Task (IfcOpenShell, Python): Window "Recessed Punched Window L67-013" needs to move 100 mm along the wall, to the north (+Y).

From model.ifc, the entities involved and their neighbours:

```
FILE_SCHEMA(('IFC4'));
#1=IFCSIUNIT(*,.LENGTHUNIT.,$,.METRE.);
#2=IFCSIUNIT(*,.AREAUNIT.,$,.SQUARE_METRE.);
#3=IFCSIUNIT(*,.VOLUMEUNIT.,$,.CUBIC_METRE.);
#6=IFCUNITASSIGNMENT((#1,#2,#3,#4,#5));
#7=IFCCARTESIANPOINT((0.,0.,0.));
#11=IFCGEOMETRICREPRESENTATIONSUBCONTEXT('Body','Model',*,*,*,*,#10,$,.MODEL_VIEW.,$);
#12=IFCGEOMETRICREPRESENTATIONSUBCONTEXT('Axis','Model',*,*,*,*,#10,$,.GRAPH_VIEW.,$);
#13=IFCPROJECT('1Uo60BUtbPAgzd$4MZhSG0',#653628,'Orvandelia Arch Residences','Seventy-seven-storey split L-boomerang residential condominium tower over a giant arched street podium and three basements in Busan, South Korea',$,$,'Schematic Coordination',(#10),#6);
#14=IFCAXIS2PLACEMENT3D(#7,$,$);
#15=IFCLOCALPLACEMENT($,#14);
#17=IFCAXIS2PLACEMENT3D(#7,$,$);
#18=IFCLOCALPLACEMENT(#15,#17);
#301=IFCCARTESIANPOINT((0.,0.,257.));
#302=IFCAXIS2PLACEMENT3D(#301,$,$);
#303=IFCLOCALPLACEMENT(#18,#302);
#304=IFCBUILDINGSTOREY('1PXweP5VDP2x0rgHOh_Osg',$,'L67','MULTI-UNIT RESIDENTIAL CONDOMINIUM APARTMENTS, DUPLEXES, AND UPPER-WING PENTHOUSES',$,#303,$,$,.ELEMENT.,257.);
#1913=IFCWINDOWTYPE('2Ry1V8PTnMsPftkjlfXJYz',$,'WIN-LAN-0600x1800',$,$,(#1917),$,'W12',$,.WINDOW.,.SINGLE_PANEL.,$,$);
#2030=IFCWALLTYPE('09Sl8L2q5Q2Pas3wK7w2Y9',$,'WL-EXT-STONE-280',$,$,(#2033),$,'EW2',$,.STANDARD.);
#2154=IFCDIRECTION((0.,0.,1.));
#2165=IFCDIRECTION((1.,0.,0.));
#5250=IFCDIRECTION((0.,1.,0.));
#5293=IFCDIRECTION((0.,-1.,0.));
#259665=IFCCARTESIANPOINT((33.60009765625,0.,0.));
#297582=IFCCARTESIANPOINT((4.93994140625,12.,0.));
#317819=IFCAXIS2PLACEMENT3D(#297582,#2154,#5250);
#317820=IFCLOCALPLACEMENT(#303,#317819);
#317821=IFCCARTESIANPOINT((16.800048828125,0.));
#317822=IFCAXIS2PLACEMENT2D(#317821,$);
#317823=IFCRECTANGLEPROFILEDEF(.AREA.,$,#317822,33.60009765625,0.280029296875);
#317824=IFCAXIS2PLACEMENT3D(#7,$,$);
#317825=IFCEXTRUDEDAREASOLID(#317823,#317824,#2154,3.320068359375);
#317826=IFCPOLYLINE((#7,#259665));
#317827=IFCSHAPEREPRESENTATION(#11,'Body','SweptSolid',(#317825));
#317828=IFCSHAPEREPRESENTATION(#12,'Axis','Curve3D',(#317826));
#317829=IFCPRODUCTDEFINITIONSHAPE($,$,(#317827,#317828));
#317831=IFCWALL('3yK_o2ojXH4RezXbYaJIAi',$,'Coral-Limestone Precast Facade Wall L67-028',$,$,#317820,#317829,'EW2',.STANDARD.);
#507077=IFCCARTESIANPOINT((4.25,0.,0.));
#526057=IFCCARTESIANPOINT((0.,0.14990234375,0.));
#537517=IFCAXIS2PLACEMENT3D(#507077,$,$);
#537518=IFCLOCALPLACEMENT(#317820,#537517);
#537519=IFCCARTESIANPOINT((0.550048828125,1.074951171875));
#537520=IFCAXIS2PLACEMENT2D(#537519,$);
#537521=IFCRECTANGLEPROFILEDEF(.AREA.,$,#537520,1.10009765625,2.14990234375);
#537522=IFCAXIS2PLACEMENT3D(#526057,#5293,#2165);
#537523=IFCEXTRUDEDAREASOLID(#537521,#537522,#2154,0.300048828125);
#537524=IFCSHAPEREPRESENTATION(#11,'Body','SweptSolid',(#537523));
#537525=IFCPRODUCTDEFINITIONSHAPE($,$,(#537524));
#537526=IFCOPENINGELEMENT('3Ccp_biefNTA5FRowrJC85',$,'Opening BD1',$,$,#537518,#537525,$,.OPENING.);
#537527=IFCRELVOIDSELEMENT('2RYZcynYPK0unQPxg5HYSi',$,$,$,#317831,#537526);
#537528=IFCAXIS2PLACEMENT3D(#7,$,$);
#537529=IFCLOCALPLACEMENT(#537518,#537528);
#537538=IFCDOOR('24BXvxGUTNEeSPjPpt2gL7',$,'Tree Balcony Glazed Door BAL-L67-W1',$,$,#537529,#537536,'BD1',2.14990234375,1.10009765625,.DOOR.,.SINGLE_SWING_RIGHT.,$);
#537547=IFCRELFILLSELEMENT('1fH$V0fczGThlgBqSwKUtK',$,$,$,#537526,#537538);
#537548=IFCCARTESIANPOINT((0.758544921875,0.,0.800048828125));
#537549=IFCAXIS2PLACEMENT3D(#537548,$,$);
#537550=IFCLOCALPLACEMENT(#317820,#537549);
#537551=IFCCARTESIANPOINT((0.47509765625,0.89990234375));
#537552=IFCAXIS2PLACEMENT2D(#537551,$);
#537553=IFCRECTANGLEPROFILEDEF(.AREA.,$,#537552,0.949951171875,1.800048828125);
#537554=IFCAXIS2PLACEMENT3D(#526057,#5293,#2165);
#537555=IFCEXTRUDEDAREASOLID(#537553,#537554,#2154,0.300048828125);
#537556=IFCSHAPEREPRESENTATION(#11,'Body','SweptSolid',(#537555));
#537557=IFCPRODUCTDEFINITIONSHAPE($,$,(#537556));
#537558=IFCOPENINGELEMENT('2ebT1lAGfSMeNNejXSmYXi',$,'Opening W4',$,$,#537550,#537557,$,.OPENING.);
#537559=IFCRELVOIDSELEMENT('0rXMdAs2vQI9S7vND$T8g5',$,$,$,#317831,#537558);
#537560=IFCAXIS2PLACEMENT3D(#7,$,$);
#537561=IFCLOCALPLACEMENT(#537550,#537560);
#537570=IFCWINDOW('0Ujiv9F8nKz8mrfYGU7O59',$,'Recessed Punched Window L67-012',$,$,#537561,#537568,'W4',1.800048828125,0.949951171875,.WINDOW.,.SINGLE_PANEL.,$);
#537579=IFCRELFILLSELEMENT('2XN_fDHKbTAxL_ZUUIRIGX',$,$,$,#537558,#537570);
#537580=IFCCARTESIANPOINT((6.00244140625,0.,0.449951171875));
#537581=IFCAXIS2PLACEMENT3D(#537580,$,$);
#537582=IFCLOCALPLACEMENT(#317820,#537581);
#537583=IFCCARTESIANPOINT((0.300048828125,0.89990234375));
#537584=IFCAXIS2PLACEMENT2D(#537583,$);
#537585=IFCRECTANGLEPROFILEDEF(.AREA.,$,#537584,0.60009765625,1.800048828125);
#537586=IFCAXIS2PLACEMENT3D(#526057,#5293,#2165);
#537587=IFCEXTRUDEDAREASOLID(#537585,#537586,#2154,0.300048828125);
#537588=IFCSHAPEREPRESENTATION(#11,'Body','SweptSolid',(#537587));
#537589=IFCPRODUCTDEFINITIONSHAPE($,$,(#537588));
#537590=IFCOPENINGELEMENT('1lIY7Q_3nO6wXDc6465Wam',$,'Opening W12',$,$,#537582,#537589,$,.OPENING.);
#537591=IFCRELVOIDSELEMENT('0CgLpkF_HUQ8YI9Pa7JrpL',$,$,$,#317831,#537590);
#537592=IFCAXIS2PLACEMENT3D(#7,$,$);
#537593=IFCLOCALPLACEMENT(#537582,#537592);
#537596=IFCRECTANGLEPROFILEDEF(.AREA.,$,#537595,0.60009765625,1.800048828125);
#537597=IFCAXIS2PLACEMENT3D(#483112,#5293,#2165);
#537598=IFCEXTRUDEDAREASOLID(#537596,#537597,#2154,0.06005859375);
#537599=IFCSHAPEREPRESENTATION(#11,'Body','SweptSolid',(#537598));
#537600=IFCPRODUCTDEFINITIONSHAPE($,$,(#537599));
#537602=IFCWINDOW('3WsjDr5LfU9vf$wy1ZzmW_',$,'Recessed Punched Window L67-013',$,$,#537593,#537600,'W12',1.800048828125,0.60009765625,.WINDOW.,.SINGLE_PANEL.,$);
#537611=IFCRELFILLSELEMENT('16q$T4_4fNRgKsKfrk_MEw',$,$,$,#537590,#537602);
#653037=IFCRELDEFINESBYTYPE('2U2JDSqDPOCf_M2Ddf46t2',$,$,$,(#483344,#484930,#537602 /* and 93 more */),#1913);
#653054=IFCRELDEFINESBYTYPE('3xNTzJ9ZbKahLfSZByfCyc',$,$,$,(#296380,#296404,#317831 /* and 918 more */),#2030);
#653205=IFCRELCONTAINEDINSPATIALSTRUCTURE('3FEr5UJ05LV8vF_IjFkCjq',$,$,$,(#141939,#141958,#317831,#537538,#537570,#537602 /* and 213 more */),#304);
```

```python
import ifcopenshell
import ifcopenshell.api.geometry
import ifcopenshell.util.placement

model = ifcopenshell.open("model.ifc")

window = model.by_guid("3WsjDr5LfU9vf$wy1ZzmW_")
opening = window.FillsVoids[0].RelatingOpeningElement
wall = opening.VoidsElements[0].RelatingBuildingElement

wall_matrix = ifcopenshell.util.placement.get_local_placement(wall.ObjectPlacement)
shift = wall_matrix[:3, 0] * 0.1
before = ifcopenshell.util.placement.get_local_placement(window.ObjectPlacement)[:3, 3].copy()

# The window is placed relative to its opening, so it follows when the opening moves.
matrix = ifcopenshell.util.placement.get_local_placement(opening.ObjectPlacement)
matrix[:3, 3] += shift
ifcopenshell.api.geometry.edit_object_placement(
    model, product=opening, matrix=matrix, is_si=False, should_transform_children=True
)

after = ifcopenshell.util.placement.get_local_placement(window.ObjectPlacement)[:3, 3]
print("window moved by", (after - before).round(3) + 0.0)

model.write("model_edited.ifc")
```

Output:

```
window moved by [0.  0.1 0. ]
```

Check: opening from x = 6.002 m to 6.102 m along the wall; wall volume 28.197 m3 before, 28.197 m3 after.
